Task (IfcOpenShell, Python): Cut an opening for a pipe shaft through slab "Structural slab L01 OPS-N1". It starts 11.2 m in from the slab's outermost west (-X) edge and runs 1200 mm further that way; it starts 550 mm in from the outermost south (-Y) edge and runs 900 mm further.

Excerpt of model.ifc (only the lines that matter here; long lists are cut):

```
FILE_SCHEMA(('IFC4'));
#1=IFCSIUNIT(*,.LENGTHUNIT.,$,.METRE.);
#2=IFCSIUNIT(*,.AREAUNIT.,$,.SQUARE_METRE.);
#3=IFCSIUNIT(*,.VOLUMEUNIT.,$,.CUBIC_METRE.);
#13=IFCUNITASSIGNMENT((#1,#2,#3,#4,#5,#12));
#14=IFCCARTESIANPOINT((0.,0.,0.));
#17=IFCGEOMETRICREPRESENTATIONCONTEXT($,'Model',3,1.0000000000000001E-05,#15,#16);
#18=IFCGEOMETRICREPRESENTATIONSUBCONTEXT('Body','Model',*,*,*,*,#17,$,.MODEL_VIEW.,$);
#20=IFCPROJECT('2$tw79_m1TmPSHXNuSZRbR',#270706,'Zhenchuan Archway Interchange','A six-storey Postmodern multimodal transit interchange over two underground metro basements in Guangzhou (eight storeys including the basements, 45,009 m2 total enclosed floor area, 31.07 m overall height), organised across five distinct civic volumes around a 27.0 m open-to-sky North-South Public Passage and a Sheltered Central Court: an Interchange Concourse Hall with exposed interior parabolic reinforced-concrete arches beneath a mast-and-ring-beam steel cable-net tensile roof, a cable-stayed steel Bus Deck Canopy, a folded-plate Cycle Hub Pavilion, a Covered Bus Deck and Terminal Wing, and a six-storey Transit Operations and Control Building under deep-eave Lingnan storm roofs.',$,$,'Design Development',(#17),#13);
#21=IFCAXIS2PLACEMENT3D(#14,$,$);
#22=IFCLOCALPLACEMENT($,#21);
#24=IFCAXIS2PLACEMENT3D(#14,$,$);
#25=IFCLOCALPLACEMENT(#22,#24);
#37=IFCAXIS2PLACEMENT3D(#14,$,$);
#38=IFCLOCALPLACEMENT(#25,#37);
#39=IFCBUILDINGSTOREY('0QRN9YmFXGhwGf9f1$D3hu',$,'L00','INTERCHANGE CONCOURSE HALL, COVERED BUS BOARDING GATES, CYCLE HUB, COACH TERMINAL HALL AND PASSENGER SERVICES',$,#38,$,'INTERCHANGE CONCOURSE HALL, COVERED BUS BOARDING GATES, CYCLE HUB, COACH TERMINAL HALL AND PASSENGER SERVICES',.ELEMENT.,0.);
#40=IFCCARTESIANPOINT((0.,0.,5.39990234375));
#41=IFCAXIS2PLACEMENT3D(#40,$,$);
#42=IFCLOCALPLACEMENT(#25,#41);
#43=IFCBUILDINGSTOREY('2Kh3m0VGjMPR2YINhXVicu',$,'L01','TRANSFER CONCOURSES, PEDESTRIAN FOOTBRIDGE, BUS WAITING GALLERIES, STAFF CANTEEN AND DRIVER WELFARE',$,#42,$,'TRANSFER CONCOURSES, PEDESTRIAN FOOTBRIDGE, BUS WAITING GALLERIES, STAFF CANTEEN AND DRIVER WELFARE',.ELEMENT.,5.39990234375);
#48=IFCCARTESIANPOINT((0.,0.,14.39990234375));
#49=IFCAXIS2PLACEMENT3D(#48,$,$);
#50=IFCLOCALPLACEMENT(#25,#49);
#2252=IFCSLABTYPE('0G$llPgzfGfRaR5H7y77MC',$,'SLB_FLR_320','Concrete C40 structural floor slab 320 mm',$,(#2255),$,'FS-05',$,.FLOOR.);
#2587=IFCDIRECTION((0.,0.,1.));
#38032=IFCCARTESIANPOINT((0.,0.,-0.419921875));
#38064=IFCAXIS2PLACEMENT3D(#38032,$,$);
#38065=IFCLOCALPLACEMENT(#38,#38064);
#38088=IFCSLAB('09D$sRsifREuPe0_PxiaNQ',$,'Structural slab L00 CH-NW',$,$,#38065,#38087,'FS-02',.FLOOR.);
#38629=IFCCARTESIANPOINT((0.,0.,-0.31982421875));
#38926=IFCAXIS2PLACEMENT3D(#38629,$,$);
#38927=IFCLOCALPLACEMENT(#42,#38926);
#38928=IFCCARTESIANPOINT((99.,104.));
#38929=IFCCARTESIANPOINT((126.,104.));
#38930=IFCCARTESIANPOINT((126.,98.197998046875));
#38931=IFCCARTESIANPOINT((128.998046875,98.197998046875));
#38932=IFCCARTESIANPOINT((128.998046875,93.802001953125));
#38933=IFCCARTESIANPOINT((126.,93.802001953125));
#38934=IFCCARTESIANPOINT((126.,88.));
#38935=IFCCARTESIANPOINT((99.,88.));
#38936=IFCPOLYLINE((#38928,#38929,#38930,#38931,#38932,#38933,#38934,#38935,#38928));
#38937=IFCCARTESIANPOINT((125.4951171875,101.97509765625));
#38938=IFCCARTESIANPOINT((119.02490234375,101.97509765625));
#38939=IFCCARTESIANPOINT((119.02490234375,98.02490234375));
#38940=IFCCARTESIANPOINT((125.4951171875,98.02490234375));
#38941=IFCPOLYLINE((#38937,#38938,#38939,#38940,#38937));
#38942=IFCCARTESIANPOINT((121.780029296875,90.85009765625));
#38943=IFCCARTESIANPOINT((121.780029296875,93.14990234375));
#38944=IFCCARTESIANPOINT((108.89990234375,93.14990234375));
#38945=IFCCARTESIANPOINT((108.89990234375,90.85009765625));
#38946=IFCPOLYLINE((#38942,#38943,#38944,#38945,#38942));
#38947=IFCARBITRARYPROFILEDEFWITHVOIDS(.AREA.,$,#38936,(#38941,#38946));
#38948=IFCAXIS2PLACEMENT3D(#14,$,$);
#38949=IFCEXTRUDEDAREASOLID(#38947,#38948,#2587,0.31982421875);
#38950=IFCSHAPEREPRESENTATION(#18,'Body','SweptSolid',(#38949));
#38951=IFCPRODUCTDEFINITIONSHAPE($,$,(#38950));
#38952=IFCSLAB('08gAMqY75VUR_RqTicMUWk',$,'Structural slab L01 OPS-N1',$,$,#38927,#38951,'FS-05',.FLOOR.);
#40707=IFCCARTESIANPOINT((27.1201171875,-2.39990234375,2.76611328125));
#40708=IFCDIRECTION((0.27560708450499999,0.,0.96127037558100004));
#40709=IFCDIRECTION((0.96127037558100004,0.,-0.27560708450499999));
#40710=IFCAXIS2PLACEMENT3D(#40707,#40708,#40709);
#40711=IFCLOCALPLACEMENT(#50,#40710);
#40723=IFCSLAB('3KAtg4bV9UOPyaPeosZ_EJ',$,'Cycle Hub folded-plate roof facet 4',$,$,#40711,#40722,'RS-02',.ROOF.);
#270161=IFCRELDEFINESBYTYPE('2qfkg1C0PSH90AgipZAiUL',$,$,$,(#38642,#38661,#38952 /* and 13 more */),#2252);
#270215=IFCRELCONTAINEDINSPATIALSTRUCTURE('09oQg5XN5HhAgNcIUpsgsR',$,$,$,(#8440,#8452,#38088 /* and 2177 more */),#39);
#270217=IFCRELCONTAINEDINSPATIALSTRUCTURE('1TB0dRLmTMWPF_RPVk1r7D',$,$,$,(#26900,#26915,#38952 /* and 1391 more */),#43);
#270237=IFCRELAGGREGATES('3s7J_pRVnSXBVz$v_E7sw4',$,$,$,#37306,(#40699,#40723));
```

```python
import numpy as np
import ifcopenshell
import ifcopenshell.api.feature
import ifcopenshell.api.geometry
import ifcopenshell.api.root
import ifcopenshell.geom
import ifcopenshell.util.placement
import ifcopenshell.util.representation
import ifcopenshell.util.shape
import ifcopenshell.util.unit

model = ifcopenshell.open("model.ifc")
unit_scale = ifcopenshell.util.unit.calculate_unit_scale(model)
settings = ifcopenshell.geom.settings()


def volume(element):
    """Net volume in cubic metres, openings subtracted."""
    shape = ifcopenshell.geom.create_shape(settings, element)
    return ifcopenshell.util.shape.get_volume(shape.geometry)


slab = model.by_guid("08gAMqY75VUR_RqTicMUWk")
before = volume(slab)

# Extent in the slab's own axes, in metres. The edges named are its -X and -Y sides.
slab_shape = ifcopenshell.geom.create_shape(settings, slab)
vertices = ifcopenshell.util.shape.get_vertices(slab_shape.geometry)
x_min, y_min, bottom = vertices.min(axis=0)
top = vertices[:, 2].max()

opening = ifcopenshell.api.root.create_entity(model, ifc_class="IfcOpeningElement", name="Pipe shaft opening", predefined_type="OPENING")
context = ifcopenshell.util.representation.get_context(model, "Model", "Body", "MODEL_VIEW")
width, depth = 1.2, 0.9
outline = [(0.0, 0.0), (width, 0.0), (width, depth), (0.0, depth), (0.0, 0.0)]
# Overshoot both faces by 50 mm so the cut is clean.
shape = ifcopenshell.api.geometry.add_slab_representation(
    model, context=context, depth=top - bottom + 0.1, polyline=outline
)
ifcopenshell.api.geometry.assign_representation(model, product=opening, representation=shape)

matrix = ifcopenshell.util.placement.get_local_placement(slab.ObjectPlacement)
matrix[:, 3] = matrix @ np.append(np.array([x_min + 11.2, y_min + 0.55, bottom - 0.05]) / unit_scale, 1.0)
ifcopenshell.api.geometry.edit_object_placement(model, product=opening, matrix=matrix, is_si=False)
ifcopenshell.api.feature.add_feature(model, feature=opening, element=slab)

after = volume(slab)

print(f"slab volume {before:.3f} -> {after:.3f} m3")

model.write("model_rev.ifc")
```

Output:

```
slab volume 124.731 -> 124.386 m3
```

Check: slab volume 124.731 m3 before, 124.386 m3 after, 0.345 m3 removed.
